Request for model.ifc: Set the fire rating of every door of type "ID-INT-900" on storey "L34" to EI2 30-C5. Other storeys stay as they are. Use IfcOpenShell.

First a look at what the model holds.

```python
import ifcopenshell
import ifcopenshell.util.element

model = ifcopenshell.open("model.ifc")
print(model.schema)
storey = next(s for s in model.by_type("IfcBuildingStorey") if s.Name == "L34")
doors = [e for e in ifcopenshell.util.element.get_decomposition(storey) if e.is_a("IfcDoor")]
seen = {}
for e in doors:
    element_type = ifcopenshell.util.element.get_type(e)
    key = (element_type.Name if element_type != e and element_type else None, ifcopenshell.util.element.get_pset(e, "Pset_DoorCommon", "FireRating"))
    seen[key] = seen.get(key, 0) + 1
for (name, value), count in sorted(seen.items(), key=str):
    print(count, "x", name, "|", value)
```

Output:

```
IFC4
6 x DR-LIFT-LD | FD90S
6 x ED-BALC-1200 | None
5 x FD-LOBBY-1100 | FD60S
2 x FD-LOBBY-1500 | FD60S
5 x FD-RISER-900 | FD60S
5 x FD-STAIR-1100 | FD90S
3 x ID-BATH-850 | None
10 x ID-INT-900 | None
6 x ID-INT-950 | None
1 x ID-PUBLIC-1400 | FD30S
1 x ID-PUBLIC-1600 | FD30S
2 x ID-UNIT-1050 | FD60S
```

```python
import ifcopenshell
import ifcopenshell.api.pset
import ifcopenshell.util.element

model = ifcopenshell.open("model.ifc")

storey = next(s for s in model.by_type("IfcBuildingStorey") if s.Name == "L34")
doors = [e for e in ifcopenshell.util.element.get_decomposition(storey) if e.is_a("IfcDoor")]

count = 0
for e in doors:
    element_type = ifcopenshell.util.element.get_type(e)
    if element_type in (None, e) or element_type.Name != "ID-INT-900":
        continue
    found = ifcopenshell.util.element.get_pset(e, "Pset_DoorCommon", should_inherit=False)
    if found:
        pset = model.by_id(found["id"])
        if len(ifcopenshell.util.element.get_elements_by_pset(pset)) > 1:
            pset = ifcopenshell.api.pset.unshare_pset(model, products=[e], pset=pset)[0]
    else:
        pset = ifcopenshell.api.pset.add_pset(model, product=e, name="Pset_DoorCommon")
    ifcopenshell.api.pset.edit_pset(model, pset=pset, properties={"FireRating": "EI2 30-C5"})
    count += 1

print(count, "doors updated")

model.write("model_v2.ifc")
```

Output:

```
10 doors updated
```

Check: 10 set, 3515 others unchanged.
